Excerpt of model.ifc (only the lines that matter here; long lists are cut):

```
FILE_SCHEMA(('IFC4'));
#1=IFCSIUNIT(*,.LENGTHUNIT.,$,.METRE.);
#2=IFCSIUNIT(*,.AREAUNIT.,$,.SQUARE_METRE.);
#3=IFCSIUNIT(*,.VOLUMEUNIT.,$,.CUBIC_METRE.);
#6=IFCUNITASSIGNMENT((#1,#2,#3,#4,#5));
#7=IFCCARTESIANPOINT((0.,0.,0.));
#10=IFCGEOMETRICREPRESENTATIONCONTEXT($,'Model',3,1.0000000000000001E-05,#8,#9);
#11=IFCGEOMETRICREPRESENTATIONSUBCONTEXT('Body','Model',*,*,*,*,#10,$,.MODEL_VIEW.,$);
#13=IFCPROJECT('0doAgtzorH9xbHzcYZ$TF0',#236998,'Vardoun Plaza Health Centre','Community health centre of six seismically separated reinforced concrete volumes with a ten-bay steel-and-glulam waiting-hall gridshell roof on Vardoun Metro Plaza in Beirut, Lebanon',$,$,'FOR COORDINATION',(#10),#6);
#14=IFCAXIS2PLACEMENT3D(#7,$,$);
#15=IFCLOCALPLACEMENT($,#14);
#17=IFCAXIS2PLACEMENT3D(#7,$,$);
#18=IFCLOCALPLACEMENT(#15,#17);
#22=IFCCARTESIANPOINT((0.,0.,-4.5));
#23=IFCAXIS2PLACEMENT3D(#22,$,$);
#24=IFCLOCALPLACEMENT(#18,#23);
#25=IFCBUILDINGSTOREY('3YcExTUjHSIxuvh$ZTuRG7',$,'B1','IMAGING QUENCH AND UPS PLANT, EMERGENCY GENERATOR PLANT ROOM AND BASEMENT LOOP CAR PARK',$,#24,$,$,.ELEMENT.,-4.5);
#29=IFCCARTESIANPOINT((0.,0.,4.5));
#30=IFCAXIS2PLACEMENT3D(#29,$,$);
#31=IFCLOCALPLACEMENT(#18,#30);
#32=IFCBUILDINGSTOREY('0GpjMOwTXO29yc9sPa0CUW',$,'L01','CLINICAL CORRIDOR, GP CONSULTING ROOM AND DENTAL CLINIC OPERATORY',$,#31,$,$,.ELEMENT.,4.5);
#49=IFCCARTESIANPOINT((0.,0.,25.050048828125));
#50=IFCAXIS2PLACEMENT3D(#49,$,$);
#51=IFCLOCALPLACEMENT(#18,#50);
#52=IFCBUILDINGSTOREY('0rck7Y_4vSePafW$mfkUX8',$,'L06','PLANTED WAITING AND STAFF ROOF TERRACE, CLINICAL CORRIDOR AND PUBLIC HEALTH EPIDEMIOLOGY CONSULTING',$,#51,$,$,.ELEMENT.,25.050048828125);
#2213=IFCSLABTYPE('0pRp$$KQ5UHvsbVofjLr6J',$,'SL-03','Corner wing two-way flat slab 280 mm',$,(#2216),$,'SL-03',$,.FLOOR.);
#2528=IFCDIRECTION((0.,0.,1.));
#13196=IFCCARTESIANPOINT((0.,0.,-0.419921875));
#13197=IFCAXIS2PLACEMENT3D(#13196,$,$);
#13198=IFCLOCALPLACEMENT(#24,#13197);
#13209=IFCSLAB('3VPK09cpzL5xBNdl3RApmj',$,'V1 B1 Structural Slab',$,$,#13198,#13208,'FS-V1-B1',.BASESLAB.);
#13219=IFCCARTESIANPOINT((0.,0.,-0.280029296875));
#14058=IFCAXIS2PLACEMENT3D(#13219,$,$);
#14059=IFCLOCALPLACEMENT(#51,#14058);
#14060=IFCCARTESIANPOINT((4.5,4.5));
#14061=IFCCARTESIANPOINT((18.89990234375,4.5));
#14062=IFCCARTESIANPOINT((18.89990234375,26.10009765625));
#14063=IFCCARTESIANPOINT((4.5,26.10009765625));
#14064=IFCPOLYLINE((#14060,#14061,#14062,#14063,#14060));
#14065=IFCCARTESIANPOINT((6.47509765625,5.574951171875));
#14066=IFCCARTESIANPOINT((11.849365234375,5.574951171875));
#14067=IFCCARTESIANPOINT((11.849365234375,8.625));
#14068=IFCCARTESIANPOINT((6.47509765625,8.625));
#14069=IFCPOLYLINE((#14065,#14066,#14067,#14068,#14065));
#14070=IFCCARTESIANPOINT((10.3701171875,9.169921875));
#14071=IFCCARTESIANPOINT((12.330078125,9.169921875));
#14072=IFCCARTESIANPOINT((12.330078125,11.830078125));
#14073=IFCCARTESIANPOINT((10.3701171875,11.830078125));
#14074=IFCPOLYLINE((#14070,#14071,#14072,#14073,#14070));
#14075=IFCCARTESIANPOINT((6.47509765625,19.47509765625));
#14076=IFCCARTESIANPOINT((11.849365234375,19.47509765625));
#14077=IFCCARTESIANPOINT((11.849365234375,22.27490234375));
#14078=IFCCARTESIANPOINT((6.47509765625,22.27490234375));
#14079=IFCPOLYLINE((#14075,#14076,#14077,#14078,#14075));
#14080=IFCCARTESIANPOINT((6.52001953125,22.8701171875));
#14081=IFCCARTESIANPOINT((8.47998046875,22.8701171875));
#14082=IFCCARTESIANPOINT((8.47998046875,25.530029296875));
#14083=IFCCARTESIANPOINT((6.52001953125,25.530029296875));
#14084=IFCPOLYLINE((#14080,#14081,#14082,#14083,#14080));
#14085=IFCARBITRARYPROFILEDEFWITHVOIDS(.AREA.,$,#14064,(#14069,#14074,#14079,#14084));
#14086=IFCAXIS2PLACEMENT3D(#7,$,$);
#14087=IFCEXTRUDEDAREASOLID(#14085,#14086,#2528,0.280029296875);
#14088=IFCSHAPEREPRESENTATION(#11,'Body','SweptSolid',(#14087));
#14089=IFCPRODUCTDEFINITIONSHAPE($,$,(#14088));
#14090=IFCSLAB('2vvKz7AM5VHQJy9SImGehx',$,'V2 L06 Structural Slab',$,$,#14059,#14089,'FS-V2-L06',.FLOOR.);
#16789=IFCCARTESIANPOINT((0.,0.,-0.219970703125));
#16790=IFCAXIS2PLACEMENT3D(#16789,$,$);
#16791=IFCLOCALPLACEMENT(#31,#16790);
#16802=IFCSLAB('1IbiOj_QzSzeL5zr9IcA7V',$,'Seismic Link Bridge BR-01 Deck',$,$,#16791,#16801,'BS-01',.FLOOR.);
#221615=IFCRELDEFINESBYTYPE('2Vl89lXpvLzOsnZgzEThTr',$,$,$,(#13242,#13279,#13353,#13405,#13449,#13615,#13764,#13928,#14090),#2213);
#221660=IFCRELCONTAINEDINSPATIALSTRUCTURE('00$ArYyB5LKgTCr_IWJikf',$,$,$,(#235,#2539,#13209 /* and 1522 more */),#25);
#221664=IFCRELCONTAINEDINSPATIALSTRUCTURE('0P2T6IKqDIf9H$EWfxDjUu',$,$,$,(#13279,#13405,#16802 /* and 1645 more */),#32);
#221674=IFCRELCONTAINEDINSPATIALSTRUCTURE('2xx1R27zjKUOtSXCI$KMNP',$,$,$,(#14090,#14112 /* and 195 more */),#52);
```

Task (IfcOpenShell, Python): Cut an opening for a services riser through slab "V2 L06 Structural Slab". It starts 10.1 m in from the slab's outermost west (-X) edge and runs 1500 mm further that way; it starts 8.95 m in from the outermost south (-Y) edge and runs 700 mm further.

```python
import numpy as np
import ifcopenshell
import ifcopenshell.api.feature
import ifcopenshell.api.geometry
import ifcopenshell.api.root
import ifcopenshell.geom
import ifcopenshell.util.placement
import ifcopenshell.util.representation
import ifcopenshell.util.shape
import ifcopenshell.util.unit

model = ifcopenshell.open("model.ifc")
unit_scale = ifcopenshell.util.unit.calculate_unit_scale(model)
settings = ifcopenshell.geom.settings()


def volume(element):
    """Net volume in cubic metres, openings subtracted."""
    shape = ifcopenshell.geom.create_shape(settings, element)
    return ifcopenshell.util.shape.get_volume(shape.geometry)


slab = model.by_guid("2vvKz7AM5VHQJy9SImGehx")
before = volume(slab)

# Extent in the slab's own axes, in metres. The edges named are its -X and -Y sides.
slab_shape = ifcopenshell.geom.create_shape(settings, slab)
vertices = ifcopenshell.util.shape.get_vertices(slab_shape.geometry)
x_min, y_min, bottom = vertices.min(axis=0)
top = vertices[:, 2].max()

opening = ifcopenshell.api.root.create_entity(model, ifc_class="IfcOpeningElement", name="Services riser opening", predefined_type="OPENING")
context = ifcopenshell.util.representation.get_context(model, "Model", "Body", "MODEL_VIEW")
width, depth = 1.5, 0.7
outline = [(0.0, 0.0), (width, 0.0), (width, depth), (0.0, depth), (0.0, 0.0)]
# Overshoot both faces by 50 mm so the cut is clean.
shape = ifcopenshell.api.geometry.add_slab_representation(
    model, context=context, depth=top - bottom + 0.1, polyline=outline
)
ifcopenshell.api.geometry.assign_representation(model, product=opening, representation=shape)

matrix = ifcopenshell.util.placement.get_local_placement(slab.ObjectPlacement)
matrix[:, 3] = matrix @ np.append(np.array([x_min + 10.1, y_min + 8.95, bottom - 0.05]) / unit_scale, 1.0)
ifcopenshell.api.geometry.edit_object_placement(model, product=opening, matrix=matrix, is_si=False)
ifcopenshell.api.feature.add_feature(model, feature=opening, element=slab)

after = volume(slab)

print(f"slab volume {before:.3f} -> {after:.3f} m3")

model.write("model-out.ifc")
```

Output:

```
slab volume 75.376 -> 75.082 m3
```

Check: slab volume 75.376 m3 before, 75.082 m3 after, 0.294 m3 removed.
